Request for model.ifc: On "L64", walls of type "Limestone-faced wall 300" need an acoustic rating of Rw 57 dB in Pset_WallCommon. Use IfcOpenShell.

First a look at what the model holds.

```python
import ifcopenshell
import ifcopenshell.util.element

model = ifcopenshell.open("model.ifc")
print(model.schema)
storey = next(s for s in model.by_type("IfcBuildingStorey") if s.Name == "L64")
walls = [e for e in ifcopenshell.util.element.get_decomposition(storey) if e.is_a("IfcWall")]
seen = {}
for e in walls:
    element_type = ifcopenshell.util.element.get_type(e)
    key = (element_type.Name if element_type != e and element_type else None, ifcopenshell.util.element.get_pset(e, "Pset_WallCommon", "AcousticRating"))
    seen[key] = seen.get(key, 0) + 1
for (name, value), count in sorted(seen.items(), key=str):
    print(count, "x", name, "|", value)
```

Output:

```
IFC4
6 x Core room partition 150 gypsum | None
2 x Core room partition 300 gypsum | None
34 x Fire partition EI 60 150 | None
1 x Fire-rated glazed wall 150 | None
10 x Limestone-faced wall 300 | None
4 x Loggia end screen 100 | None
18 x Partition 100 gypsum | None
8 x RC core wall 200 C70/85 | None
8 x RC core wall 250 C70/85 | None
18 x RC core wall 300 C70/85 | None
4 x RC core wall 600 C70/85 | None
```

```python
import ifcopenshell
import ifcopenshell.api.pset
import ifcopenshell.util.element

model = ifcopenshell.open("model.ifc")

storey = next(s for s in model.by_type("IfcBuildingStorey") if s.Name == "L64")
walls = [e for e in ifcopenshell.util.element.get_decomposition(storey) if e.is_a("IfcWall")]

count = 0
for e in walls:
    element_type = ifcopenshell.util.element.get_type(e)
    if element_type in (None, e) or element_type.Name != "Limestone-faced wall 300":
        continue
    found = ifcopenshell.util.element.get_pset(e, "Pset_WallCommon", should_inherit=False)
    if found:
        pset = model.by_id(found["id"])
        if len(ifcopenshell.util.element.get_elements_by_pset(pset)) > 1:
            pset = ifcopenshell.api.pset.unshare_pset(model, products=[e], pset=pset)[0]
    else:
        pset = ifcopenshell.api.pset.add_pset(model, product=e, name="Pset_WallCommon")
    ifcopenshell.api.pset.edit_pset(model, pset=pset, properties={"AcousticRating": "Rw 57 dB"})
    count += 1

print(count, "walls updated")

model.write("model-out.ifc")
```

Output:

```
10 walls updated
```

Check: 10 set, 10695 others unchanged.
